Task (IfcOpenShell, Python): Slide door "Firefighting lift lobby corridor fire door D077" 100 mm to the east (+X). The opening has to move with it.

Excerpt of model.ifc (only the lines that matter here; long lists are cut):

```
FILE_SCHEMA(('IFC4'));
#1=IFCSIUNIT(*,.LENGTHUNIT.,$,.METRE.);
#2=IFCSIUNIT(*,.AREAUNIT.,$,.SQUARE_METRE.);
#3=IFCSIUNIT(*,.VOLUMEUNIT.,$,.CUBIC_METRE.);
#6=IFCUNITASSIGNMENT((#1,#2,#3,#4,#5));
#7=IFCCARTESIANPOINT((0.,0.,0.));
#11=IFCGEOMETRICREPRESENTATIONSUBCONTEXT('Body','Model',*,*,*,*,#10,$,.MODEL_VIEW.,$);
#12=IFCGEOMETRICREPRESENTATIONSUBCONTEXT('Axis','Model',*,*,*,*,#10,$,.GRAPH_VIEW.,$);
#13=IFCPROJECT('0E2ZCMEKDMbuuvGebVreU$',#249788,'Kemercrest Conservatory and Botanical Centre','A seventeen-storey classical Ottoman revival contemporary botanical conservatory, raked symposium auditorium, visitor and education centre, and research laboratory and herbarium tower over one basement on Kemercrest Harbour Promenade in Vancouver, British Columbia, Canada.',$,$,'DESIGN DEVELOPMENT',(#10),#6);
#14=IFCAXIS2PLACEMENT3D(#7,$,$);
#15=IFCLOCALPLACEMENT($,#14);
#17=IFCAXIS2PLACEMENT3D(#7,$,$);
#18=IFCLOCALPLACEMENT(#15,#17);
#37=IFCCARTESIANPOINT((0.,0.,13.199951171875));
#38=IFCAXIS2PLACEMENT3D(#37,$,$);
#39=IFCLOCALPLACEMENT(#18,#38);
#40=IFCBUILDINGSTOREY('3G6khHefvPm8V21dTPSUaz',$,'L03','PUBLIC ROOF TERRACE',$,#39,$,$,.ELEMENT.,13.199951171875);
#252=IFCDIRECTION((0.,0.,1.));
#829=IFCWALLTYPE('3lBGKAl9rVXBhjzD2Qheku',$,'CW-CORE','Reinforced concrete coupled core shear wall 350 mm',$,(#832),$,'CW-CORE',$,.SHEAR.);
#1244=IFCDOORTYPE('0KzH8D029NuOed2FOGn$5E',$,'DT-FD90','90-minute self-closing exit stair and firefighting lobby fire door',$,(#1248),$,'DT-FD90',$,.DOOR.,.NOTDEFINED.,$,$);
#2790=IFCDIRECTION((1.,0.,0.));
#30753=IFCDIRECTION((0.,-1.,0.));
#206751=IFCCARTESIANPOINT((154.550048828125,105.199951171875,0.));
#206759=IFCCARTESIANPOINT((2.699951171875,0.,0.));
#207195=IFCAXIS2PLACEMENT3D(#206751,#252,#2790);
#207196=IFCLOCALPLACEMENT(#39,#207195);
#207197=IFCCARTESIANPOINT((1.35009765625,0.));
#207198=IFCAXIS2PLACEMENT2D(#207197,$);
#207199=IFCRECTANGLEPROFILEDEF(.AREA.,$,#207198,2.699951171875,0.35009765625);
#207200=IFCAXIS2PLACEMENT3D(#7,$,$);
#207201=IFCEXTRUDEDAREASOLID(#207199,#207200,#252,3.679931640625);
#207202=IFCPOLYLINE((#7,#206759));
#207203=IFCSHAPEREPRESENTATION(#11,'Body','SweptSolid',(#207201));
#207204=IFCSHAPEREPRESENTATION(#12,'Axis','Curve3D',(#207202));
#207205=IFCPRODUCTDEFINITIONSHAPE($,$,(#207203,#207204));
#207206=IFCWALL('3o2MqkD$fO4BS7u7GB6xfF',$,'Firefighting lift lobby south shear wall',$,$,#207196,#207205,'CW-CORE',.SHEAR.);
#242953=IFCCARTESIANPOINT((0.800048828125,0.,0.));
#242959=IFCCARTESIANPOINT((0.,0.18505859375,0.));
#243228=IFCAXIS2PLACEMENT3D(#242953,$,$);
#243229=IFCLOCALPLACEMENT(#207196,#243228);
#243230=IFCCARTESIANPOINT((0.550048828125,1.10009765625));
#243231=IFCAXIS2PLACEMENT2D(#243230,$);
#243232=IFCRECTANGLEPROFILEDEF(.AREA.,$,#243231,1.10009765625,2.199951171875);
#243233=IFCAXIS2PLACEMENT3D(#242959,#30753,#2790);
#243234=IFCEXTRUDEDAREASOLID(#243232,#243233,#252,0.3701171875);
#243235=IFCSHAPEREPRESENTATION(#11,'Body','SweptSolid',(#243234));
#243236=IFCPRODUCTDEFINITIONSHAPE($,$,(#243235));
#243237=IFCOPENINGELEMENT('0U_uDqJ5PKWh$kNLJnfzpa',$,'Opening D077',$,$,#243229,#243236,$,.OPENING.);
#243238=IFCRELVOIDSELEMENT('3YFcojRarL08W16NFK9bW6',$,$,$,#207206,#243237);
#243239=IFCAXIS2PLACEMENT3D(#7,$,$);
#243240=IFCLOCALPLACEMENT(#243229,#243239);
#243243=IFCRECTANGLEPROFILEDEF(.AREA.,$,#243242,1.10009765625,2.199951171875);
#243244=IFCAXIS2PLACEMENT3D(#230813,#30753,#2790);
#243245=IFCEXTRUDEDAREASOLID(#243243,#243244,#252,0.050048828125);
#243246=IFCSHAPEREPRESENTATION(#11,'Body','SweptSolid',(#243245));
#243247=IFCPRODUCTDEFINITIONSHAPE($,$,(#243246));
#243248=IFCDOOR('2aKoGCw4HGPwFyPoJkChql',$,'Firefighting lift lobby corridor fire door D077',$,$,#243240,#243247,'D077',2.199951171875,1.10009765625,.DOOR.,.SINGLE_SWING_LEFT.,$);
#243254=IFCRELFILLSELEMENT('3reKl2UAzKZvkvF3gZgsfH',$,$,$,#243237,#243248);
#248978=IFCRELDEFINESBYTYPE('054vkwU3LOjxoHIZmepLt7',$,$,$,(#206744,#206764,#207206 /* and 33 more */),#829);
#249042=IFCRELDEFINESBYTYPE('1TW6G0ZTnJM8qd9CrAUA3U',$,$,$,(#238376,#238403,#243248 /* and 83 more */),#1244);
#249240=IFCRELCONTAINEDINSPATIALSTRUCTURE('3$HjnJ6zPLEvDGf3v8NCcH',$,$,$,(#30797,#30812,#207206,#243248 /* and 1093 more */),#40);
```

```python
import ifcopenshell
import ifcopenshell.api.geometry
import ifcopenshell.util.placement

model = ifcopenshell.open("model.ifc")

door = model.by_guid("2aKoGCw4HGPwFyPoJkChql")
opening = door.FillsVoids[0].RelatingOpeningElement
wall = opening.VoidsElements[0].RelatingBuildingElement

wall_matrix = ifcopenshell.util.placement.get_local_placement(wall.ObjectPlacement)
shift = wall_matrix[:3, 0] * 0.1
before = ifcopenshell.util.placement.get_local_placement(door.ObjectPlacement)[:3, 3].copy()

# The door is placed relative to its opening, so it follows when the opening moves.
matrix = ifcopenshell.util.placement.get_local_placement(opening.ObjectPlacement)
matrix[:3, 3] += shift
ifcopenshell.api.geometry.edit_object_placement(
    model, product=opening, matrix=matrix, is_si=False, should_transform_children=True
)

after = ifcopenshell.util.placement.get_local_placement(door.ObjectPlacement)[:3, 3]
print("door moved by", (after - before).round(3) + 0.0)

model.write("model_edited.ifc")
```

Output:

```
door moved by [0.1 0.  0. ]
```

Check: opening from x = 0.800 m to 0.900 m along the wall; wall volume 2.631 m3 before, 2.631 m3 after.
